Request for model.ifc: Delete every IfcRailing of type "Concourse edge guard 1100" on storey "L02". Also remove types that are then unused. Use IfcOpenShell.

First a look at what the model holds.

```python
import ifcopenshell
import ifcopenshell.util.element

model = ifcopenshell.open("model.ifc")
print(model.schema)
storey = next(s for s in model.by_type("IfcBuildingStorey") if s.Name == "L02")
railings = [e for e in ifcopenshell.util.element.get_decomposition(storey) if e.is_a("IfcRailing")]
seen = {}
for e in railings:
    element_type = ifcopenshell.util.element.get_type(e)
    name = element_type.Name if element_type not in (None, e) else None
    seen[name] = seen.get(name, 0) + 1
for name, count in sorted(seen.items(), key=str):
    print(count, "x", name)
```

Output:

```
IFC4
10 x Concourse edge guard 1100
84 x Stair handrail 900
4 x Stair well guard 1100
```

```python
import ifcopenshell
import ifcopenshell.api.root
import ifcopenshell.util.element

model = ifcopenshell.open("model.ifc")

storey = next(s for s in model.by_type("IfcBuildingStorey") if s.Name == "L02")
railings = [e for e in ifcopenshell.util.element.get_decomposition(storey) if e.is_a("IfcRailing")]
targets = [e for e in railings if (t := ifcopenshell.util.element.get_type(e)) not in (None, e) and t.Name == "Concourse edge guard 1100"]
types = {ifcopenshell.util.element.get_type(e) for e in targets} - {None, *targets}

for e in targets:
    ifcopenshell.api.root.remove_product(model, product=e)
print(len(targets), "removed")

unused = [t for t in types if not ifcopenshell.util.element.get_types(t)]
for t in unused:
    ifcopenshell.api.root.remove_product(model, product=t)
print(len(unused), "unused types removed")

model.write("model_edited.ifc")
```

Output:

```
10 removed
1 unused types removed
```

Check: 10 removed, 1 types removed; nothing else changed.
